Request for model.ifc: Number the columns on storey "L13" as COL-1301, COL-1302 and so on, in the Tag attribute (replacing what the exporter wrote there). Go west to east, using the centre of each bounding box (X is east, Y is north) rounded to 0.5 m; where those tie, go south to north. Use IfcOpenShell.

First a look at what the model holds.

```python
import ifcopenshell
import ifcopenshell.util.element
import ifcopenshell.util.placement

model = ifcopenshell.open("model.ifc")
print(model.schema)
storey = next(s for s in model.by_type("IfcBuildingStorey") if s.Name == "L13")
columns = [e for e in ifcopenshell.util.element.get_decomposition(storey) if e.is_a("IfcColumn")]
for e in sorted(columns, key=lambda e: e.id()):
    origin = ifcopenshell.util.placement.get_local_placement(e.ObjectPlacement)[:3, 3]
    print(e.id(), e.Tag, e.Name, origin.round(2) + 0.0, sep=" | ")
```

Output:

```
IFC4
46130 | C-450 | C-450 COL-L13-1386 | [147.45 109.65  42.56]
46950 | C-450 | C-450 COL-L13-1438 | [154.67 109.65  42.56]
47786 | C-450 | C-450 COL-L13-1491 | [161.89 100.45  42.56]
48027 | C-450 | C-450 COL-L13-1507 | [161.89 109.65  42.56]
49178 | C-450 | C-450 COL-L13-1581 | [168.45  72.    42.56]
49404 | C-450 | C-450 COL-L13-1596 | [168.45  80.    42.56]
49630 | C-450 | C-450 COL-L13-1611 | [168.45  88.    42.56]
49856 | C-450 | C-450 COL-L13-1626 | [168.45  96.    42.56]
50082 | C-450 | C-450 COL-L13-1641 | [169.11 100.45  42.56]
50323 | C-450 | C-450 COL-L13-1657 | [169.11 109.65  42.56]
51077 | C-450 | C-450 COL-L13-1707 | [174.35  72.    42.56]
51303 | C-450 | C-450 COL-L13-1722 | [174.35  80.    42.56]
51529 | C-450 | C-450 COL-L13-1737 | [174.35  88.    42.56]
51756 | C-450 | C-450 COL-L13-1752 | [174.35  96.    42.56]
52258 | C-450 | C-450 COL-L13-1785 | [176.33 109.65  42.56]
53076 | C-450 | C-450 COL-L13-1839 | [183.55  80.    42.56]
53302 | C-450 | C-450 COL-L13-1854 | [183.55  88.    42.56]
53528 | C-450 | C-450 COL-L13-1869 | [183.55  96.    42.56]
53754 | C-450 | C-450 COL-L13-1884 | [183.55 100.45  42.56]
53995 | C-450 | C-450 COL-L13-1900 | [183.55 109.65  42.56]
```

```python
import ifcopenshell
import ifcopenshell.geom
import ifcopenshell.util.element
import ifcopenshell.util.shape

model = ifcopenshell.open("model.ifc")
settings = ifcopenshell.geom.settings()
settings.set("use-world-coords", True)


def centre(element):
    shape = ifcopenshell.geom.create_shape(settings, element)
    return ifcopenshell.util.shape.get_bbox_centroid(shape.geometry)


storey = next(s for s in model.by_type("IfcBuildingStorey") if s.Name == "L13")
columns = [e for e in ifcopenshell.util.element.get_decomposition(storey) if e.is_a("IfcColumn")]

# Insertion points can sit at a corner or the storey origin, so sort by the geometry (in metres).
centres = {e: centre(e) for e in columns}
columns.sort(key=lambda e: (round(centres[e][0] / 0.5), centres[e][1]))

for i, e in enumerate(columns, start=1):
    number = f"COL-13{i:02d}"
    e.Tag = number
    print(e.id(), number)

model.write("model-out.ifc")
```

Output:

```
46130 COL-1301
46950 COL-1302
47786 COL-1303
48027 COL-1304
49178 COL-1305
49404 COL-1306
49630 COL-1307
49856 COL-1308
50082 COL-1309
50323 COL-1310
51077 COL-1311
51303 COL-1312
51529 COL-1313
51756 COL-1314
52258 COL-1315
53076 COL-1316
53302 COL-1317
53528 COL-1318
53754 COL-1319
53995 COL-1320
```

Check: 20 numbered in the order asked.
